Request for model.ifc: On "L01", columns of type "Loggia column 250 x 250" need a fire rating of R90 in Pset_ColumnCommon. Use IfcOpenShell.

First a look at what the model holds.

```python
import ifcopenshell
import ifcopenshell.util.element

model = ifcopenshell.open("model.ifc")
print(model.schema)
storey = next(s for s in model.by_type("IfcBuildingStorey") if s.Name == "L01")
columns = [e for e in ifcopenshell.util.element.get_decomposition(storey) if e.is_a("IfcColumn")]
seen = {}
for e in columns:
    element_type = ifcopenshell.util.element.get_type(e)
    key = (element_type.Name if element_type != e and element_type else None, ifcopenshell.util.element.get_pset(e, "Pset_ColumnCommon", "FireRating"))
    seen[key] = seen.get(key, 0) + 1
for (name, value), count in sorted(seen.items(), key=str):
    print(count, "x", name, "|", value)
```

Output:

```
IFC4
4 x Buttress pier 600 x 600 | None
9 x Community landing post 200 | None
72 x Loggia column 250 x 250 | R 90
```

```python
import ifcopenshell
import ifcopenshell.api.pset
import ifcopenshell.util.element

model = ifcopenshell.open("model.ifc")

storey = next(s for s in model.by_type("IfcBuildingStorey") if s.Name == "L01")
columns = [e for e in ifcopenshell.util.element.get_decomposition(storey) if e.is_a("IfcColumn")]

count = 0
for e in columns:
    element_type = ifcopenshell.util.element.get_type(e)
    if element_type in (None, e) or element_type.Name != "Loggia column 250 x 250":
        continue
    # add_pset returns the element's existing set when there is one.
    pset = ifcopenshell.api.pset.add_pset(model, product=e, name="Pset_ColumnCommon")
    ifcopenshell.api.pset.edit_pset(model, pset=pset, properties={"FireRating": "R90"})
    count += 1

print(count, "columns updated")

model.write("model_edited.ifc")
```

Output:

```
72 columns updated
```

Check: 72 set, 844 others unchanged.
